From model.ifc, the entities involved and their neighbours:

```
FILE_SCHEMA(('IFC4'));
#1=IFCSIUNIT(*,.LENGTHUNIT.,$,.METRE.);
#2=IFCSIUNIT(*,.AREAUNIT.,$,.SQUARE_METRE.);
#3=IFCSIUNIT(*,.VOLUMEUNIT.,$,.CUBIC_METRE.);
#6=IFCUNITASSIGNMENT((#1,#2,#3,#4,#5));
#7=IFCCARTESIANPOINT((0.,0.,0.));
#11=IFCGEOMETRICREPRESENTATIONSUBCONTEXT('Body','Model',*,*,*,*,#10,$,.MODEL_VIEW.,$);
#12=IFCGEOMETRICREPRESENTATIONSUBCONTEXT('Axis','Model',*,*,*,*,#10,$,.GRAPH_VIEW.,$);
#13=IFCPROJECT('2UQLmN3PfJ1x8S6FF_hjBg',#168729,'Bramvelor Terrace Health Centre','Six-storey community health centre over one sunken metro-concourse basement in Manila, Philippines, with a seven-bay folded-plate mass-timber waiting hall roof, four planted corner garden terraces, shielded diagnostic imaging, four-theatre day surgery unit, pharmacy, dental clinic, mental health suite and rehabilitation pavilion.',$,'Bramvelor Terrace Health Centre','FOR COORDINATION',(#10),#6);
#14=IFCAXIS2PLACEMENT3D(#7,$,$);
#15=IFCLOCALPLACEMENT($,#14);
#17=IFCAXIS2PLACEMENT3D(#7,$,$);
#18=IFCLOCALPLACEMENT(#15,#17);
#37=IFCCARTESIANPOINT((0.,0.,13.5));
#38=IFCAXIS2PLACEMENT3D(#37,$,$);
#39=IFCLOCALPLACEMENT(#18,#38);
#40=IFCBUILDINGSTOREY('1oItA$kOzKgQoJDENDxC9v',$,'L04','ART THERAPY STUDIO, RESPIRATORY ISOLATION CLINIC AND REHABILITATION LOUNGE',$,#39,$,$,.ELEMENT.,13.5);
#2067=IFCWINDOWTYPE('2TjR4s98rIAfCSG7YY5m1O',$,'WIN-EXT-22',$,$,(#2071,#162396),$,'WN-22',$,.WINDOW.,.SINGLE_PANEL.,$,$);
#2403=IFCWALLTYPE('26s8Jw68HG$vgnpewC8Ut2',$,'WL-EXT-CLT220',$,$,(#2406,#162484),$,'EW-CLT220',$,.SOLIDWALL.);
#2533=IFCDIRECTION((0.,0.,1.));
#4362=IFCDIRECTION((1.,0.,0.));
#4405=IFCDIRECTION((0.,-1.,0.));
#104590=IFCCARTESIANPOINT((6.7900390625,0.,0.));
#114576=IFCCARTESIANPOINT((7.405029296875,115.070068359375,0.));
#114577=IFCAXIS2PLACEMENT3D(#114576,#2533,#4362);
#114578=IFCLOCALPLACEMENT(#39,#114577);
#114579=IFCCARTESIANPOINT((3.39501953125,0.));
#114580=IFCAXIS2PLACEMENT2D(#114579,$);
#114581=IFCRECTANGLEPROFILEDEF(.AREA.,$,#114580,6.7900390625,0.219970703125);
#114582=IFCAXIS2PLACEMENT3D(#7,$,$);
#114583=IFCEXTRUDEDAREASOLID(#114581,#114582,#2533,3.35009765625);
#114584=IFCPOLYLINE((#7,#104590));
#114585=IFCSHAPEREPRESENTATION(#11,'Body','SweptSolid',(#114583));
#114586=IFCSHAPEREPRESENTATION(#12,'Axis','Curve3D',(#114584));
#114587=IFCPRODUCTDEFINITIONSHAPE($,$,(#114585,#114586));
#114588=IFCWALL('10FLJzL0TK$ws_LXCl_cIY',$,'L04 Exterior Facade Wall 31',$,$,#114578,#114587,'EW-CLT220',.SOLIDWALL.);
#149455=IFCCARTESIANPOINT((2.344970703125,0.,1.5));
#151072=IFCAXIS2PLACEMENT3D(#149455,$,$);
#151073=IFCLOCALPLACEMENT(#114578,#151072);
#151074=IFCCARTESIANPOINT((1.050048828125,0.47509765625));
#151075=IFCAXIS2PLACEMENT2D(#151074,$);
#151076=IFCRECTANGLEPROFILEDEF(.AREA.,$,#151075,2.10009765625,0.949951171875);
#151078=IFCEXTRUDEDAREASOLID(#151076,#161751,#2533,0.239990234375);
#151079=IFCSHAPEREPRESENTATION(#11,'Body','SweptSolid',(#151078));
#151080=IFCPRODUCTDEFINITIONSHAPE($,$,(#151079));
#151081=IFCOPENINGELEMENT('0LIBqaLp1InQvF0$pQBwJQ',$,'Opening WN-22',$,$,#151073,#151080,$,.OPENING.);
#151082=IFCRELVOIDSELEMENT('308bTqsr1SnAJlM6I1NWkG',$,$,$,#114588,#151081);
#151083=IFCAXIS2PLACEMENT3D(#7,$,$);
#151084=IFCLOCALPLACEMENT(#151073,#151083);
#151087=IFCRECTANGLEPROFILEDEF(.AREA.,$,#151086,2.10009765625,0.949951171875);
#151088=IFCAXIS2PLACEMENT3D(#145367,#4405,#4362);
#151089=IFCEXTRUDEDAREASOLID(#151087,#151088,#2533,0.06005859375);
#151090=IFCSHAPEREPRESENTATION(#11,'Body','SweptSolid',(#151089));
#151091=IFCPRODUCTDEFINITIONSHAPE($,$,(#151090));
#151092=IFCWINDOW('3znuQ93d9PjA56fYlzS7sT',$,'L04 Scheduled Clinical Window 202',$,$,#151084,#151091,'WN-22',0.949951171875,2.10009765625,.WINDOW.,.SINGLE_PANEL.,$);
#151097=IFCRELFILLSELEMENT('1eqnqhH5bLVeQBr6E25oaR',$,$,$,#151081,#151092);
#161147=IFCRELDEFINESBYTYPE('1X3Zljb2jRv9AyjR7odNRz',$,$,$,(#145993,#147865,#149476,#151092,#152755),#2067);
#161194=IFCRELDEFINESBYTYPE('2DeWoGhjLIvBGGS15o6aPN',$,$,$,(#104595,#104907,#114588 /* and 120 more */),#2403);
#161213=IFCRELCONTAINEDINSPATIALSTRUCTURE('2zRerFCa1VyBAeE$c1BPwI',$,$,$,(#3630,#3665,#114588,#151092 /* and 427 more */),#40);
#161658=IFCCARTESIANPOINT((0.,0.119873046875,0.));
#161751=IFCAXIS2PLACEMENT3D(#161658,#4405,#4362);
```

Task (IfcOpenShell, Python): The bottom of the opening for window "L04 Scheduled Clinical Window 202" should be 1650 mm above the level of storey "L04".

```python
import numpy as np
import ifcopenshell
import ifcopenshell.api.geometry
import ifcopenshell.geom
import ifcopenshell.util.element
import ifcopenshell.util.placement
import ifcopenshell.util.shape
import ifcopenshell.util.unit

model = ifcopenshell.open("model.ifc")
unit_scale = ifcopenshell.util.unit.calculate_unit_scale(model)

window = model.by_id(151092)
opening = window.FillsVoids[0].RelatingOpeningElement
storey = ifcopenshell.util.element.get_container(window, ifc_class="IfcBuildingStorey")
level = ifcopenshell.util.placement.get_local_placement(storey.ObjectPlacement)[2, 3]

# The opening's origin need not be at the sill, so measure its lowest point.
shape = ifcopenshell.geom.create_shape(ifcopenshell.geom.settings(), opening)
bottom = ifcopenshell.util.shape.get_shape_bottom_elevation(shape, shape.geometry) / unit_scale
dz = level + 1.65 / unit_scale - bottom

shift = np.array([0.0, 0.0, dz])
# The window is placed relative to its opening, so it follows when the opening moves.
matrix = ifcopenshell.util.placement.get_local_placement(opening.ObjectPlacement)
matrix[:3, 3] += shift
ifcopenshell.api.geometry.edit_object_placement(
    model, product=opening, matrix=matrix, is_si=False, should_transform_children=True
)

print(f"moved by {dz * unit_scale:+.3f} m")

model.write("model_updated.ifc")
```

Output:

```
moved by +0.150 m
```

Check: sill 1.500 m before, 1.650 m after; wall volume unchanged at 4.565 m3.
